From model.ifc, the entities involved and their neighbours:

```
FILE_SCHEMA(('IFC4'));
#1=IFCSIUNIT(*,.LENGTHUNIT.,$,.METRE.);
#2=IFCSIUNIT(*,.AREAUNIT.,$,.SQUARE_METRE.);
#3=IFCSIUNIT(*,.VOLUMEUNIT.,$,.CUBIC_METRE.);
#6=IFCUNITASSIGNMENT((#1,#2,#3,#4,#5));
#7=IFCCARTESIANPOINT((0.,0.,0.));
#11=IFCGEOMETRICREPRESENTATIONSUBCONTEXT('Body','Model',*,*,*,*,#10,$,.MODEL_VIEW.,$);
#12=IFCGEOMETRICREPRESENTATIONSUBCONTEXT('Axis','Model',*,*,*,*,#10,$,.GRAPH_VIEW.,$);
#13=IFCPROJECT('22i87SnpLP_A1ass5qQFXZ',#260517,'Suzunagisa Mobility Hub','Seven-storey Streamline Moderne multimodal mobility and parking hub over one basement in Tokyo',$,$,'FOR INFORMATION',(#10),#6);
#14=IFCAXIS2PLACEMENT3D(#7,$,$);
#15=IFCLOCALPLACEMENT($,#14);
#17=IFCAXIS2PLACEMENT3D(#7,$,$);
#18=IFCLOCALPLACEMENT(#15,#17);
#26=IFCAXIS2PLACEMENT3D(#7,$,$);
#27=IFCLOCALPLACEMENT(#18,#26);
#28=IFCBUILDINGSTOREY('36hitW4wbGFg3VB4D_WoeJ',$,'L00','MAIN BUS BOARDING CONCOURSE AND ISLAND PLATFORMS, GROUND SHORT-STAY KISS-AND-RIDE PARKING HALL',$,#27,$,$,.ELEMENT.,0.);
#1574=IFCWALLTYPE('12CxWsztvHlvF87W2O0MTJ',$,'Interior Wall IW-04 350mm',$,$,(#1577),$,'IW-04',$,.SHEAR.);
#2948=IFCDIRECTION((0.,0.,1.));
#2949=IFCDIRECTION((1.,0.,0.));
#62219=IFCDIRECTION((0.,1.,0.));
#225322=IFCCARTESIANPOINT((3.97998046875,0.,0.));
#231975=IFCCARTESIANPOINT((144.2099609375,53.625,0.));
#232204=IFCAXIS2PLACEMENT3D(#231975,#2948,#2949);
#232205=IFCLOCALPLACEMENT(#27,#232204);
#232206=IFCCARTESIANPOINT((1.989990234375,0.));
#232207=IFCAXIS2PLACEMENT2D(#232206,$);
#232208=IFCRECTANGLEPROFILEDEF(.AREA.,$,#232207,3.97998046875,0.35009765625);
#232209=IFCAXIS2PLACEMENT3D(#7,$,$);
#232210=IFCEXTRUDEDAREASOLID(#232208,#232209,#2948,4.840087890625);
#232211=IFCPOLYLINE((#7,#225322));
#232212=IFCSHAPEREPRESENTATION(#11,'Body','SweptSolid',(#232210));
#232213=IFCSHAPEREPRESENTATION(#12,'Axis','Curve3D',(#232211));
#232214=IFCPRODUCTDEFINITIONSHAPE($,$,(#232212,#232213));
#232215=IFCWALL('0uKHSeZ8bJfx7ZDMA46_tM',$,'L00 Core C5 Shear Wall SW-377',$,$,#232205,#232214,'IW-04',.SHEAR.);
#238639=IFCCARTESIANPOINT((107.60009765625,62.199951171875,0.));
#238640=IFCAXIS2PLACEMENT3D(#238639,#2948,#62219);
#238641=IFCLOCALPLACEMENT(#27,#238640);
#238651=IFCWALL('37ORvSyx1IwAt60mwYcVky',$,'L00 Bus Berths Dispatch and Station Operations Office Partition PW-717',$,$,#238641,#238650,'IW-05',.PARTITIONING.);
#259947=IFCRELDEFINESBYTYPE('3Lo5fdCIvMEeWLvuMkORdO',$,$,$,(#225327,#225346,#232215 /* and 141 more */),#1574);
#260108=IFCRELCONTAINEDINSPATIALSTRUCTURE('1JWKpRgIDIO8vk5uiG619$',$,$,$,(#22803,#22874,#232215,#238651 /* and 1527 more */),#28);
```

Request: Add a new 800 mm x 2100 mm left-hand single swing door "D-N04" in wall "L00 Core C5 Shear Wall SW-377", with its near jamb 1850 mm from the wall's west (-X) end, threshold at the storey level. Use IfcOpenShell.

```python
import numpy as np
import ifcopenshell
import ifcopenshell.api.feature
import ifcopenshell.api.geometry
import ifcopenshell.api.root
import ifcopenshell.api.spatial
import ifcopenshell.geom
import ifcopenshell.util.element
import ifcopenshell.util.placement
import ifcopenshell.util.representation
import ifcopenshell.util.shape
import ifcopenshell.util.unit

model = ifcopenshell.open("model.ifc")
unit_scale = ifcopenshell.util.unit.calculate_unit_scale(model)
settings = ifcopenshell.geom.settings()


def volume(element):
    """Net volume in cubic metres, openings subtracted."""
    shape = ifcopenshell.geom.create_shape(settings, element)
    return ifcopenshell.util.shape.get_volume(shape.geometry)


wall = model.by_guid("0uKHSeZ8bJfx7ZDMA46_tM")
storey = ifcopenshell.util.element.get_container(wall, ifc_class="IfcBuildingStorey")
context = ifcopenshell.util.representation.get_context(model, "Model", "Body", "MODEL_VIEW")
before = volume(wall)

width, height, from_end, sill = 0.8, 2.1, 1.85, 0.0  # metres

# The wall runs along its own X axis, and the end named is its -X end.
wall_shape = ifcopenshell.geom.create_shape(settings, wall)
x, y, z = ifcopenshell.util.shape.get_vertices(wall_shape.geometry).T
start = x.min() + from_end
face, thickness = float(y.min()), float(y.max() - y.min())
wall_matrix = ifcopenshell.util.placement.get_local_placement(wall.ObjectPlacement)
level = ifcopenshell.util.placement.get_local_placement(storey.ObjectPlacement)[2, 3]


def in_wall(x, y):
    """Placement at x, y metres in the wall's axes, at sill height."""
    matrix = wall_matrix.copy()
    matrix[:, 3] = wall_matrix @ np.array([x / unit_scale, y / unit_scale, 0.0, 1.0])
    matrix[2, 3] = level + sill / unit_scale
    return matrix


# Opening: a box that overshoots both wall faces by 50 mm.
opening = ifcopenshell.api.root.create_entity(model, ifc_class="IfcOpeningElement", predefined_type="OPENING")
box = ifcopenshell.api.geometry.add_wall_representation(
    model, context=context, length=width, height=height, thickness=thickness + 0.1
)
ifcopenshell.api.geometry.assign_representation(model, product=opening, representation=box)
ifcopenshell.api.geometry.edit_object_placement(model, product=opening, matrix=in_wall(start, face - 0.05), is_si=False)
ifcopenshell.api.feature.add_feature(model, feature=opening, element=wall)

door = ifcopenshell.api.root.create_entity(model, ifc_class="IfcDoor", name="D-N04", predefined_type="DOOR")
door.OverallWidth, door.OverallHeight = width / unit_scale, height / unit_scale
door.OperationType = "SINGLE_SWING_LEFT"
body = ifcopenshell.api.geometry.add_door_representation(
    model,
    context=context,
    overall_width=door.OverallWidth,
    overall_height=door.OverallHeight,
    operation_type="SINGLE_SWING_LEFT",
    lining_properties={"LiningDepth": thickness / unit_scale, "ThresholdDepth": thickness / unit_scale},
)
ifcopenshell.api.geometry.assign_representation(model, product=door, representation=body)
ifcopenshell.api.spatial.assign_container(model, products=[door], relating_structure=storey)
ifcopenshell.api.feature.add_filling(model, opening=opening, element=door)

# The lining spans the wall, so the door starts at the wall face.
ifcopenshell.api.geometry.edit_object_placement(model, product=door, matrix=in_wall(start, face), is_si=False)

after = volume(wall)

print(f"wall volume {before:.3f} -> {after:.3f} m3")

model.write("model-out.ifc")
```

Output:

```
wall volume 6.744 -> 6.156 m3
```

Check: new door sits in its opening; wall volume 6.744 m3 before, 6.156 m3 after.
